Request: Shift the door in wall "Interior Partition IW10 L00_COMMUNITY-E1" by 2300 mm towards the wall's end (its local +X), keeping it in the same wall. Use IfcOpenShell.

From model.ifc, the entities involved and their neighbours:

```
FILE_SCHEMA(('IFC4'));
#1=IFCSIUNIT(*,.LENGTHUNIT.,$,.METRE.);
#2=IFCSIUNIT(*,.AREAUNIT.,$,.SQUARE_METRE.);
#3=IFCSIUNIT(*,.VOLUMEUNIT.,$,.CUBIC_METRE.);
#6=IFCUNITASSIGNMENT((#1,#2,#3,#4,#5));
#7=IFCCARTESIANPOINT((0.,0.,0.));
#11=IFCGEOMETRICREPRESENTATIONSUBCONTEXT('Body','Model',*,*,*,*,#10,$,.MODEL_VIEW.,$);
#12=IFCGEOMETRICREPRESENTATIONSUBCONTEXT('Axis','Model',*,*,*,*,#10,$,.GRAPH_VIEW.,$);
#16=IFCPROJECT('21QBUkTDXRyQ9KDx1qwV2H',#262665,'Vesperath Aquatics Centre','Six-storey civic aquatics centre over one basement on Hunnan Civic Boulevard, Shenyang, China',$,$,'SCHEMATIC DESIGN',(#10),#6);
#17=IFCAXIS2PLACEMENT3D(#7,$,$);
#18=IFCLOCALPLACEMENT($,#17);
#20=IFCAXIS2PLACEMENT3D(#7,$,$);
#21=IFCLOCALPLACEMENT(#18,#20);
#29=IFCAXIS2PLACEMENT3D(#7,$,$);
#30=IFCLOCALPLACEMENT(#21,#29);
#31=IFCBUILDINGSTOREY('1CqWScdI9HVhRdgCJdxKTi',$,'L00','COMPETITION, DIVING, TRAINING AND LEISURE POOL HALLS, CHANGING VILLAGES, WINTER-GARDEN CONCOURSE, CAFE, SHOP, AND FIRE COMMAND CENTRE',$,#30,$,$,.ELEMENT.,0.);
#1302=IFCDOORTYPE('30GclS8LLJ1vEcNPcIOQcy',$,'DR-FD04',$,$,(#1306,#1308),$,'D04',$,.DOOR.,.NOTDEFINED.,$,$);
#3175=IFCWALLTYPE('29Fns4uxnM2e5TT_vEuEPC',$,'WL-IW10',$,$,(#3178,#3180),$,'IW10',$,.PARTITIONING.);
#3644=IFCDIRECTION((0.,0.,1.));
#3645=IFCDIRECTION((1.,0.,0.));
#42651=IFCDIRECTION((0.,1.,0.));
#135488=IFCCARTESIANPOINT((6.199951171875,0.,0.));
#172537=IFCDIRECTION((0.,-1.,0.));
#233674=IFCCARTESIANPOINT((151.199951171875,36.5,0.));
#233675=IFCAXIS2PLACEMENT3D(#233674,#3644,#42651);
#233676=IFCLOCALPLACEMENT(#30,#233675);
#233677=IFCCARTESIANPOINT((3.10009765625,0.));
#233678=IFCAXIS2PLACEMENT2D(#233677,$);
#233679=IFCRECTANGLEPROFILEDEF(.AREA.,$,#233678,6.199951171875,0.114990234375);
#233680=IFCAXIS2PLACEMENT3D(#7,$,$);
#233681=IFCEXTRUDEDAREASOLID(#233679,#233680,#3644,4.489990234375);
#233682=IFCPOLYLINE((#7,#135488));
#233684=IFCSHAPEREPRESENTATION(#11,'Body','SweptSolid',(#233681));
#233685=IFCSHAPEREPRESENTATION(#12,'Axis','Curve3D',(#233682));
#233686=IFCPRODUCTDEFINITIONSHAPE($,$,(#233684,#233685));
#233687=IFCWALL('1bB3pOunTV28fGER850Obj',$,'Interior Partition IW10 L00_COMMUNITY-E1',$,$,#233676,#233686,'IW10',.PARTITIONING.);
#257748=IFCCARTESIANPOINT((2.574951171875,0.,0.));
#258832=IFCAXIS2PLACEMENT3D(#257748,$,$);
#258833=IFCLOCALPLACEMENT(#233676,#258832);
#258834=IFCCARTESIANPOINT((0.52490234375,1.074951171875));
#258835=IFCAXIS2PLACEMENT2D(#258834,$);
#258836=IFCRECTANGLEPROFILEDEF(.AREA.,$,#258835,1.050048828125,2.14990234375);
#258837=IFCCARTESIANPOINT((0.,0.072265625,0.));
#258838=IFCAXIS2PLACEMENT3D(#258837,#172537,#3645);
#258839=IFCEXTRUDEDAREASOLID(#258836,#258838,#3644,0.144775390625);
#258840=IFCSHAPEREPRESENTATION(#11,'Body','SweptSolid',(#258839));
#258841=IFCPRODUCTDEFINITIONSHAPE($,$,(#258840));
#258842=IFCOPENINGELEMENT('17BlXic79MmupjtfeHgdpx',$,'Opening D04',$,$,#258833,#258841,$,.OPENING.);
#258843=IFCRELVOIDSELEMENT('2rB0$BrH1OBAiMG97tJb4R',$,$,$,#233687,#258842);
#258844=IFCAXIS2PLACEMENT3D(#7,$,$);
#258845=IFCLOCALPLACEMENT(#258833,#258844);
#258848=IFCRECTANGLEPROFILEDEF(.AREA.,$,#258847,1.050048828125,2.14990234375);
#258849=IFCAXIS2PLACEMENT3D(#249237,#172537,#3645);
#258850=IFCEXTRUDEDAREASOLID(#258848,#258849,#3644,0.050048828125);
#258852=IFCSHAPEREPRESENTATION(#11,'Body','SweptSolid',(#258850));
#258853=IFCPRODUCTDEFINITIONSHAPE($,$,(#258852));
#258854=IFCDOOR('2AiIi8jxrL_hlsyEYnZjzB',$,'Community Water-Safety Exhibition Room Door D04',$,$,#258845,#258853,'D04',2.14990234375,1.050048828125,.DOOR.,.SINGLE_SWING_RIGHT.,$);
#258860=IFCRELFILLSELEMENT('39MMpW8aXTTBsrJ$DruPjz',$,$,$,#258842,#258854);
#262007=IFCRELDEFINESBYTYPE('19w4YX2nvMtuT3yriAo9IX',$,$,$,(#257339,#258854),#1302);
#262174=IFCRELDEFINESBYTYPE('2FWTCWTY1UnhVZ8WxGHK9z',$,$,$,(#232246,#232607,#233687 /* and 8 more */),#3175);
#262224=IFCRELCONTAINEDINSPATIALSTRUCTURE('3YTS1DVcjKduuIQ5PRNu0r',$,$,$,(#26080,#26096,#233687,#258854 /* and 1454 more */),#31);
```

```python
import ifcopenshell
import ifcopenshell.api.geometry
import ifcopenshell.util.placement
import ifcopenshell.util.unit

model = ifcopenshell.open("model.ifc")
unit_scale = ifcopenshell.util.unit.calculate_unit_scale(model)

door = model.by_guid("2AiIi8jxrL_hlsyEYnZjzB")
opening = door.FillsVoids[0].RelatingOpeningElement
wall = opening.VoidsElements[0].RelatingBuildingElement

wall_matrix = ifcopenshell.util.placement.get_local_placement(wall.ObjectPlacement)
shift = wall_matrix[:3, 0] * 2.3 / unit_scale
before = ifcopenshell.util.placement.get_local_placement(door.ObjectPlacement)[:3, 3].copy()

# The door is placed relative to its opening, so it follows when the opening moves.
matrix = ifcopenshell.util.placement.get_local_placement(opening.ObjectPlacement)
matrix[:3, 3] += shift
ifcopenshell.api.geometry.edit_object_placement(
    model, product=opening, matrix=matrix, is_si=False, should_transform_children=True
)

after = ifcopenshell.util.placement.get_local_placement(door.ObjectPlacement)[:3, 3]
print("door moved by", (after - before).round(3) + 0.0)

model.write("model-out.ifc")
```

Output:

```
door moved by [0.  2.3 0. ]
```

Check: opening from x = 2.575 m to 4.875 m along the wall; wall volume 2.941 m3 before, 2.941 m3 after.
